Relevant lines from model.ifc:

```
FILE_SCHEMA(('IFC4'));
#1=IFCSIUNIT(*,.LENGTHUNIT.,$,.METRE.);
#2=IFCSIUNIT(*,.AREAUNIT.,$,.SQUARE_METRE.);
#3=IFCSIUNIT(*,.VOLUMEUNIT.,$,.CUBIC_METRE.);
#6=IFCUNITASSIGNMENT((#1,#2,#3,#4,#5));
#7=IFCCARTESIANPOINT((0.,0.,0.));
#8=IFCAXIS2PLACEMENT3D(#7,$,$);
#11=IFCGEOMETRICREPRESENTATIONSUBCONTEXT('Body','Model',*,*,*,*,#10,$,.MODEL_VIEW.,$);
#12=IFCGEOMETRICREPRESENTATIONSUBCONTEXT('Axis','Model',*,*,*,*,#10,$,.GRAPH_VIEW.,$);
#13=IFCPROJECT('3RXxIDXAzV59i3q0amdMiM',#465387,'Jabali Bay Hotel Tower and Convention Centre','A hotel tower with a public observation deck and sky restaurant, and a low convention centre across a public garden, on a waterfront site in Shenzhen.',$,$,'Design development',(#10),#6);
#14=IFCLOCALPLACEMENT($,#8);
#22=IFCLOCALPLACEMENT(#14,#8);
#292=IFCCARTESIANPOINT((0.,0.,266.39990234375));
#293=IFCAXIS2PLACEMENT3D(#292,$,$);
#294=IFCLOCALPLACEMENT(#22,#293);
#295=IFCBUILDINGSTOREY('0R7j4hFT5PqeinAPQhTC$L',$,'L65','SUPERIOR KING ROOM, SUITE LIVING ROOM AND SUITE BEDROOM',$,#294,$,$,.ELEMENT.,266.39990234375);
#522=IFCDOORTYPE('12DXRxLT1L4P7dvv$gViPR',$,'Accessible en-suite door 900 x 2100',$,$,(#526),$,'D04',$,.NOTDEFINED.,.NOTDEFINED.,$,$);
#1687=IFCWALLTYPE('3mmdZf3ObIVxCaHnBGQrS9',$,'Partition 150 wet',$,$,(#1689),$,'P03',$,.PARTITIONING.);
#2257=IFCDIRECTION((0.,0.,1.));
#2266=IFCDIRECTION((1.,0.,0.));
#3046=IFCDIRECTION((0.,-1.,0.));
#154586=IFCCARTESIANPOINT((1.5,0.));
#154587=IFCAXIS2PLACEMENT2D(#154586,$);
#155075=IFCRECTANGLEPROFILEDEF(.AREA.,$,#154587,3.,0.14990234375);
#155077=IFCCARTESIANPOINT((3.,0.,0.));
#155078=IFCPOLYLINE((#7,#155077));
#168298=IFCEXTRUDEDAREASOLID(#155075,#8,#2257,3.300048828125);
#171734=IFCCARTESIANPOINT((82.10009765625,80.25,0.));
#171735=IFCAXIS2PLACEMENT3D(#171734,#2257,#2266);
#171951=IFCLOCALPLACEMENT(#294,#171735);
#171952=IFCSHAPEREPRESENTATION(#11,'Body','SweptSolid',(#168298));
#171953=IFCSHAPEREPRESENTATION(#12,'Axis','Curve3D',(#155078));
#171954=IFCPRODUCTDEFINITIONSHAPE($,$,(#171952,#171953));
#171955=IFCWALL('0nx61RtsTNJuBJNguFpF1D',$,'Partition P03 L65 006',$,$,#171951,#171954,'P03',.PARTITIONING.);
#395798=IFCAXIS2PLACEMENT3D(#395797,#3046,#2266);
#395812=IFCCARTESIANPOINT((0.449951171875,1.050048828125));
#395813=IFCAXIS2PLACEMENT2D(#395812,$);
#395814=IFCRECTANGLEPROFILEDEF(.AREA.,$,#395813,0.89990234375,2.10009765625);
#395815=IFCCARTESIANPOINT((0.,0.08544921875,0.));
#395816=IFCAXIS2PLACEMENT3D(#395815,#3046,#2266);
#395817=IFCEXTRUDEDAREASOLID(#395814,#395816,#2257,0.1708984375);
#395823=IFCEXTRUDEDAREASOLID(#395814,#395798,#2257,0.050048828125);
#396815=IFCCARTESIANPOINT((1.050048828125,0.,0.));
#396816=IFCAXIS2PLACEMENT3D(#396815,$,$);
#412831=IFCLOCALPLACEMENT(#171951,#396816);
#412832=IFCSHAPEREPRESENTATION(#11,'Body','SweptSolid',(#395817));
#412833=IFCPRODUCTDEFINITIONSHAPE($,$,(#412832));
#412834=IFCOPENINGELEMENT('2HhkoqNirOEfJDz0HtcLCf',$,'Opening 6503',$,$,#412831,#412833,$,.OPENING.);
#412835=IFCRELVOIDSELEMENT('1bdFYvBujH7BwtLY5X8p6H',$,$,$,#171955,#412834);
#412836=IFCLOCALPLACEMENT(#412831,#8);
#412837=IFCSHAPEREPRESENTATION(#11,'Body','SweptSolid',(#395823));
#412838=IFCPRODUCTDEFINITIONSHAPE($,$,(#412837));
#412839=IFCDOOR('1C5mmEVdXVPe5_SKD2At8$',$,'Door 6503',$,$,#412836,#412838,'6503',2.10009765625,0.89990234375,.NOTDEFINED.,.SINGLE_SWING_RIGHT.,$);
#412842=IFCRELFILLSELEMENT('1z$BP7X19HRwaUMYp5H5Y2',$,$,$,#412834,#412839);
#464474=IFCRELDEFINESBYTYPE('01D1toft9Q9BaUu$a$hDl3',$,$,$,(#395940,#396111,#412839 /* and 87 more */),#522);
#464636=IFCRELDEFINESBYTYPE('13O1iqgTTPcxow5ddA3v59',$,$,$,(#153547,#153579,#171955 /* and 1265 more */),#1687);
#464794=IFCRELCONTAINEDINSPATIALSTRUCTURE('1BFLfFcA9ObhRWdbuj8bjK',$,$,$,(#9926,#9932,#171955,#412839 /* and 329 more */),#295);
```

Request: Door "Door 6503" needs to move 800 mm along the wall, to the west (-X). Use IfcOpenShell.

```python
import ifcopenshell
import ifcopenshell.api.geometry
import ifcopenshell.util.placement
import ifcopenshell.util.unit

model = ifcopenshell.open("model.ifc")
unit_scale = ifcopenshell.util.unit.calculate_unit_scale(model)

door = model.by_id(412839)
opening = door.FillsVoids[0].RelatingOpeningElement
wall = opening.VoidsElements[0].RelatingBuildingElement

wall_matrix = ifcopenshell.util.placement.get_local_placement(wall.ObjectPlacement)
shift = wall_matrix[:3, 0] * -0.8 / unit_scale
before = ifcopenshell.util.placement.get_local_placement(door.ObjectPlacement)[:3, 3].copy()

# The door is placed relative to its opening, so it follows when the opening moves.
matrix = ifcopenshell.util.placement.get_local_placement(opening.ObjectPlacement)
matrix[:3, 3] += shift
ifcopenshell.api.geometry.edit_object_placement(
    model, product=opening, matrix=matrix, is_si=False, should_transform_children=True
)

after = ifcopenshell.util.placement.get_local_placement(door.ObjectPlacement)[:3, 3]
print("door moved by", (after - before).round(3) + 0.0)

model.write("model_v2.ifc")
```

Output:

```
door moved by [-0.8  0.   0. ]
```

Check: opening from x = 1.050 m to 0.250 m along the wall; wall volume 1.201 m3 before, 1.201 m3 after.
